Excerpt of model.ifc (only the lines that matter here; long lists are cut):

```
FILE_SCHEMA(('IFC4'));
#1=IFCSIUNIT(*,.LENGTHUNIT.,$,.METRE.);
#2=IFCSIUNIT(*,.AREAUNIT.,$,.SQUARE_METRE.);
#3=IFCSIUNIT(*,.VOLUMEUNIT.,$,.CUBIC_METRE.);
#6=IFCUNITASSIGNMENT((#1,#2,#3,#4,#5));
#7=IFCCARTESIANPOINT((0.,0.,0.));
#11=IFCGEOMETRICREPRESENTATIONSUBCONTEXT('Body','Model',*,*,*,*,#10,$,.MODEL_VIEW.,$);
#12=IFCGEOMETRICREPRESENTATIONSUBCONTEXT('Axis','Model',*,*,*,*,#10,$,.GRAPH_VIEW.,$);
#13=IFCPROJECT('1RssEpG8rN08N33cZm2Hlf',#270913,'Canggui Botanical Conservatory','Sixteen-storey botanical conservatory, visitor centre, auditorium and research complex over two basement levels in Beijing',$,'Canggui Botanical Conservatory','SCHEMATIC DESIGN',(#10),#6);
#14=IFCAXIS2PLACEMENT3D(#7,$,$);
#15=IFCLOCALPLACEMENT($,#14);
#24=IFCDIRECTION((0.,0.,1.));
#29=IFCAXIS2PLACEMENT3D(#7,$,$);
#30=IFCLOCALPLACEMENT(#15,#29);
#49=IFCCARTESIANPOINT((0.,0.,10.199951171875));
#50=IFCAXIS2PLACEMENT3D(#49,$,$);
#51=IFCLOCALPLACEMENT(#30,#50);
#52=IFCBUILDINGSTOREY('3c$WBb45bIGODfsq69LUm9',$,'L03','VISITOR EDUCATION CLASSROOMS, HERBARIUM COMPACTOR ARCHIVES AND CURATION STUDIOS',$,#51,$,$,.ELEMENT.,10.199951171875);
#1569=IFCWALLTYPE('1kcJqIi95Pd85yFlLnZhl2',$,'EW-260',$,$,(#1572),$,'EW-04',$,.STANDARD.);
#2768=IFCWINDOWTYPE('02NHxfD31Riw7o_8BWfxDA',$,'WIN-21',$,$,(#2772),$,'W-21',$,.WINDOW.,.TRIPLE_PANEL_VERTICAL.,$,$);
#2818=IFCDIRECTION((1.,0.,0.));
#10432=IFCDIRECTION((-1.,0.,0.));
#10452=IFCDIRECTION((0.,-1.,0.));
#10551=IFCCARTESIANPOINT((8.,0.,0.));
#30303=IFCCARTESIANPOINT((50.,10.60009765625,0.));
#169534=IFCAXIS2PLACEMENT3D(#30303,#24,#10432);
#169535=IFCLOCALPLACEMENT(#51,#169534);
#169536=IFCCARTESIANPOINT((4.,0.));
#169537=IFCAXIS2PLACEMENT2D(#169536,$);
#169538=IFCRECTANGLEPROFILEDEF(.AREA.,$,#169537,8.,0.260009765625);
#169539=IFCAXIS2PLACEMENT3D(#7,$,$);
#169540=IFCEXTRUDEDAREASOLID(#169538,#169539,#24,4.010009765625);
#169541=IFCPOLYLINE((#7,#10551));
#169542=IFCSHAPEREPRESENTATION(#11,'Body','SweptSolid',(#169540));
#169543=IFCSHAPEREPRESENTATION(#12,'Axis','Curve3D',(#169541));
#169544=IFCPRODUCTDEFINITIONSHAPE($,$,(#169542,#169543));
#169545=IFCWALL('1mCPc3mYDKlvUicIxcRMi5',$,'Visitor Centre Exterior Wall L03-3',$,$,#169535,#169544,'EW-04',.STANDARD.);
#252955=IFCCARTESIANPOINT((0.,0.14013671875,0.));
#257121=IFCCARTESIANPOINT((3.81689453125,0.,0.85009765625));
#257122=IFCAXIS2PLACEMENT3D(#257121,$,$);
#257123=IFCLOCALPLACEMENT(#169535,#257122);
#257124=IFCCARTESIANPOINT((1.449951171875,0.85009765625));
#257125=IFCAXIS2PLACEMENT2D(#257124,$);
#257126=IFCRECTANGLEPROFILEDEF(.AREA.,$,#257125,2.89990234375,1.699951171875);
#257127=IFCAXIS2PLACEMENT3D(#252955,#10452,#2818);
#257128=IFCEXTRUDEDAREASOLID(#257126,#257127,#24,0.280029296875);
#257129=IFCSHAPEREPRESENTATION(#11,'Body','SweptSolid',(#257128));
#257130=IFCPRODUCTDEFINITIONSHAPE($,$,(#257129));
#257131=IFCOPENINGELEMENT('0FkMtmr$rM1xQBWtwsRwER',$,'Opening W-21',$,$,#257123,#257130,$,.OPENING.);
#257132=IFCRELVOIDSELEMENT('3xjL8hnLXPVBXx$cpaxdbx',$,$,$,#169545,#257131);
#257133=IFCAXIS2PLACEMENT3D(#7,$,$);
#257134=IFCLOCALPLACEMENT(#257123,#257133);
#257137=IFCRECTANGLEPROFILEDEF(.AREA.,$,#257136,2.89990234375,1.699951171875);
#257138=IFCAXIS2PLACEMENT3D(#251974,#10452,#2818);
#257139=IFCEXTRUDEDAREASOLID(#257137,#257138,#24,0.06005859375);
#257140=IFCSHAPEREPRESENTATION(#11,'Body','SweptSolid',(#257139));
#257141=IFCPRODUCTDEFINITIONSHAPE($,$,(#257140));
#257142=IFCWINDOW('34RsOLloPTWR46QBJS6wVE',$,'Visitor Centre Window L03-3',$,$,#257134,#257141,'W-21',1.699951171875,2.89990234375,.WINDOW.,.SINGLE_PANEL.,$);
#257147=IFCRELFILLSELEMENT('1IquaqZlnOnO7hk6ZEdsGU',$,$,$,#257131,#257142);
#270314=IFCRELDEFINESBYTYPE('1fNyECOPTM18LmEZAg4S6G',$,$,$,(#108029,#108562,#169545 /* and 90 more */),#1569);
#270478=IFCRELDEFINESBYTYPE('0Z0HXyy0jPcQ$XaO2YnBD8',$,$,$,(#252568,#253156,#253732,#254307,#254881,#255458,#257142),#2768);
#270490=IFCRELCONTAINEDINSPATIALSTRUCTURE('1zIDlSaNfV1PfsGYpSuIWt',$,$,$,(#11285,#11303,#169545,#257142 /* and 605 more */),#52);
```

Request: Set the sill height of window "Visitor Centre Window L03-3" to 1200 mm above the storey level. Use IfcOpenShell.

```python
import numpy as np
import ifcopenshell
import ifcopenshell.api.geometry
import ifcopenshell.geom
import ifcopenshell.util.element
import ifcopenshell.util.placement
import ifcopenshell.util.shape
import ifcopenshell.util.unit

model = ifcopenshell.open("model.ifc")
unit_scale = ifcopenshell.util.unit.calculate_unit_scale(model)

window = model.by_id(257142)
opening = window.FillsVoids[0].RelatingOpeningElement
storey = ifcopenshell.util.element.get_container(window, ifc_class="IfcBuildingStorey")
level = ifcopenshell.util.placement.get_local_placement(storey.ObjectPlacement)[2, 3]

# The opening's origin need not be at the sill, so measure its lowest point.
shape = ifcopenshell.geom.create_shape(ifcopenshell.geom.settings(), opening)
bottom = ifcopenshell.util.shape.get_shape_bottom_elevation(shape, shape.geometry) / unit_scale
dz = level + 1.2 - bottom

shift = np.array([0.0, 0.0, dz])
# The window is placed relative to its opening, so it follows when the opening moves.
matrix = ifcopenshell.util.placement.get_local_placement(opening.ObjectPlacement)
matrix[:3, 3] += shift
ifcopenshell.api.geometry.edit_object_placement(
    model, product=opening, matrix=matrix, is_si=False, should_transform_children=True
)

print(f"moved by {dz * unit_scale:+.3f} m")

model.write("model_v2.ifc")
```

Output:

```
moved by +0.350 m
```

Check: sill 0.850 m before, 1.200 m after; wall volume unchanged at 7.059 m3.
